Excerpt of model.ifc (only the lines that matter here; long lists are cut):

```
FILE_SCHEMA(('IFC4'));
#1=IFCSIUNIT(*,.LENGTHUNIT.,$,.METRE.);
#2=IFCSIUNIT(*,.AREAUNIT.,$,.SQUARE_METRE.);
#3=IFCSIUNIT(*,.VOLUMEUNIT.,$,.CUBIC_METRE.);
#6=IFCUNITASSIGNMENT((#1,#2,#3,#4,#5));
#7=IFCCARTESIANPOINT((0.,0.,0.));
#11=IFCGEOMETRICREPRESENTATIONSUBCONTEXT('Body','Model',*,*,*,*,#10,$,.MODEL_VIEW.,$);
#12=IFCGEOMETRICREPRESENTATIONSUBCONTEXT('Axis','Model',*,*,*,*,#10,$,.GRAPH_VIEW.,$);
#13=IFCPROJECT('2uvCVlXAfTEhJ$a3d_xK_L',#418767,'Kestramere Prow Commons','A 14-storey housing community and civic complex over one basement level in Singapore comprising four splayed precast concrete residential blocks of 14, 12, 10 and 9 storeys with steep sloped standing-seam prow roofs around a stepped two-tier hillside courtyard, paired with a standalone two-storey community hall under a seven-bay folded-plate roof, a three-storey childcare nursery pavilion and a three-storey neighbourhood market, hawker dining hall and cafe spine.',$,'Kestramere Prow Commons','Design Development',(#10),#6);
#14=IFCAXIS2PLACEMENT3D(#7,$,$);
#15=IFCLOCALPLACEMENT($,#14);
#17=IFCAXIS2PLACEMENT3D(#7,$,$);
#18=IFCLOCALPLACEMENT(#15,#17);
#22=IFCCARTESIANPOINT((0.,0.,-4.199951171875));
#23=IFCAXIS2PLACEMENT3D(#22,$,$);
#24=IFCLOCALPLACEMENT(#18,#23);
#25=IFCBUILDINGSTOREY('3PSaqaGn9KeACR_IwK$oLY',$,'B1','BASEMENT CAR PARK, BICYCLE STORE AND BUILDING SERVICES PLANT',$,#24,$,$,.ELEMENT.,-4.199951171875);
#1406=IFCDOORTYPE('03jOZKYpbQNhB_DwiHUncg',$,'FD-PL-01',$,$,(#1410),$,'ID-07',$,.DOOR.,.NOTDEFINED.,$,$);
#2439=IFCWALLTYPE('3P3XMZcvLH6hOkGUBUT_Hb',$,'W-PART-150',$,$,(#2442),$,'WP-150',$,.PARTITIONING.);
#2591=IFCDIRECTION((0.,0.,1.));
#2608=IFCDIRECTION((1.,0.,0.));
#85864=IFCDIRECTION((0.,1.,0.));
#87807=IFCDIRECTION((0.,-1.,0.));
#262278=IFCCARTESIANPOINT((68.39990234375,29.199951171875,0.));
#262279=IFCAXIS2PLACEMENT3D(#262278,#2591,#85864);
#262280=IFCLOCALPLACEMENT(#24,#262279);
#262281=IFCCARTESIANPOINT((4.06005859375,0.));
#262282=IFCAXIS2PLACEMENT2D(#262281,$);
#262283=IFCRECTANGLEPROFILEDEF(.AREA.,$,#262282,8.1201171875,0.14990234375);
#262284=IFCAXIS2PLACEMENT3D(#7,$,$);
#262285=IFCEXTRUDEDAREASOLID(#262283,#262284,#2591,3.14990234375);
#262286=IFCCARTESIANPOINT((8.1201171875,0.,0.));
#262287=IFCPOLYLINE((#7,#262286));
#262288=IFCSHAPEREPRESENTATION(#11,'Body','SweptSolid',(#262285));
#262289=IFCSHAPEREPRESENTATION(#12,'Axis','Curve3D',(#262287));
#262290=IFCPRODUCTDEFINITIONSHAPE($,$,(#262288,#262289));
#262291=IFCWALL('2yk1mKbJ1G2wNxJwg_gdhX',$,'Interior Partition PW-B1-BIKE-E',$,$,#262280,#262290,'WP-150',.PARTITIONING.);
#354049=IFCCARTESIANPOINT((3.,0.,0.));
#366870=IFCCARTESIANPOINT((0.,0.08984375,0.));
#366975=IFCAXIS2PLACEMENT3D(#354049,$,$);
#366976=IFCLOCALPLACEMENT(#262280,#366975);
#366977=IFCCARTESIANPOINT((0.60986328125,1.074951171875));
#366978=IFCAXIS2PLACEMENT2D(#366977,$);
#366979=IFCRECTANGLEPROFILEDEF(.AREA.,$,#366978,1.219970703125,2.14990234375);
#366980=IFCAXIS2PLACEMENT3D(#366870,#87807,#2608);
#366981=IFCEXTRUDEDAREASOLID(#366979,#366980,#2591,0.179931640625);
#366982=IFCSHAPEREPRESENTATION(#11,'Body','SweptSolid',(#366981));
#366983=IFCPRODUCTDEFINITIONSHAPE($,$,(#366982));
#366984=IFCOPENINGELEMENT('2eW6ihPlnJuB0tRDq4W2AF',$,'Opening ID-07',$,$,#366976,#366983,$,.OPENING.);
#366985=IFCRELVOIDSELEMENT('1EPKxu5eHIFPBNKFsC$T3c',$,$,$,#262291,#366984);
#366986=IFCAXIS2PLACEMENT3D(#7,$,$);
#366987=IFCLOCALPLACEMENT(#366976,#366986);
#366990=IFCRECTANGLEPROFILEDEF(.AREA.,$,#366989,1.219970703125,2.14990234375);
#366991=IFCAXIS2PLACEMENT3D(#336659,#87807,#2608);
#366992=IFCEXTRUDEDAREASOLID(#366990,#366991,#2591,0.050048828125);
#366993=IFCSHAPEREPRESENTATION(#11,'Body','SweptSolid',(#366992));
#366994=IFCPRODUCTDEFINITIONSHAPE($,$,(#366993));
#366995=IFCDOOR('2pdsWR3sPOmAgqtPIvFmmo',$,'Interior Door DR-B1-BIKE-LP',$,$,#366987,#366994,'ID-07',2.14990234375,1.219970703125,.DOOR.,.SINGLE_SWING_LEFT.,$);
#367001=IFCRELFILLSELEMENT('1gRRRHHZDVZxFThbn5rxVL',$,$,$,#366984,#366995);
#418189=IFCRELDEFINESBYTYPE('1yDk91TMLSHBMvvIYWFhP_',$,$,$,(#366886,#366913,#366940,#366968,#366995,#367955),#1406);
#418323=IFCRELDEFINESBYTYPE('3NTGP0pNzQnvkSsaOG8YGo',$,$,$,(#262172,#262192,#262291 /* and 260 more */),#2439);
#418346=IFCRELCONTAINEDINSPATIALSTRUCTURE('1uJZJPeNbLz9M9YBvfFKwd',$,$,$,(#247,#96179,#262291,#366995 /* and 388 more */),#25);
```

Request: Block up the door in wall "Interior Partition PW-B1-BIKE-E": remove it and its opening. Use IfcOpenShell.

```python
import ifcopenshell
import ifcopenshell.api.feature
import ifcopenshell.api.root
import ifcopenshell.geom
import ifcopenshell.util.shape

model = ifcopenshell.open("model.ifc")
settings = ifcopenshell.geom.settings()


def volume(element):
    """Net volume in cubic metres, openings subtracted."""
    shape = ifcopenshell.geom.create_shape(settings, element)
    return ifcopenshell.util.shape.get_volume(shape.geometry)


door = model.by_id(366995)
opening = door.FillsVoids[0].RelatingOpeningElement
wall = opening.VoidsElements[0].RelatingBuildingElement
before = volume(wall)

ifcopenshell.api.root.remove_product(model, product=door)
ifcopenshell.api.feature.remove_feature(model, feature=opening)

after = volume(wall)

print(f"wall volume {before:.3f} -> {after:.3f} m3")

model.write("model_updated.ifc")
```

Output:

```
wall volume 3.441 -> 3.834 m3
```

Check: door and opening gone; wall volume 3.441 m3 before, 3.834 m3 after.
